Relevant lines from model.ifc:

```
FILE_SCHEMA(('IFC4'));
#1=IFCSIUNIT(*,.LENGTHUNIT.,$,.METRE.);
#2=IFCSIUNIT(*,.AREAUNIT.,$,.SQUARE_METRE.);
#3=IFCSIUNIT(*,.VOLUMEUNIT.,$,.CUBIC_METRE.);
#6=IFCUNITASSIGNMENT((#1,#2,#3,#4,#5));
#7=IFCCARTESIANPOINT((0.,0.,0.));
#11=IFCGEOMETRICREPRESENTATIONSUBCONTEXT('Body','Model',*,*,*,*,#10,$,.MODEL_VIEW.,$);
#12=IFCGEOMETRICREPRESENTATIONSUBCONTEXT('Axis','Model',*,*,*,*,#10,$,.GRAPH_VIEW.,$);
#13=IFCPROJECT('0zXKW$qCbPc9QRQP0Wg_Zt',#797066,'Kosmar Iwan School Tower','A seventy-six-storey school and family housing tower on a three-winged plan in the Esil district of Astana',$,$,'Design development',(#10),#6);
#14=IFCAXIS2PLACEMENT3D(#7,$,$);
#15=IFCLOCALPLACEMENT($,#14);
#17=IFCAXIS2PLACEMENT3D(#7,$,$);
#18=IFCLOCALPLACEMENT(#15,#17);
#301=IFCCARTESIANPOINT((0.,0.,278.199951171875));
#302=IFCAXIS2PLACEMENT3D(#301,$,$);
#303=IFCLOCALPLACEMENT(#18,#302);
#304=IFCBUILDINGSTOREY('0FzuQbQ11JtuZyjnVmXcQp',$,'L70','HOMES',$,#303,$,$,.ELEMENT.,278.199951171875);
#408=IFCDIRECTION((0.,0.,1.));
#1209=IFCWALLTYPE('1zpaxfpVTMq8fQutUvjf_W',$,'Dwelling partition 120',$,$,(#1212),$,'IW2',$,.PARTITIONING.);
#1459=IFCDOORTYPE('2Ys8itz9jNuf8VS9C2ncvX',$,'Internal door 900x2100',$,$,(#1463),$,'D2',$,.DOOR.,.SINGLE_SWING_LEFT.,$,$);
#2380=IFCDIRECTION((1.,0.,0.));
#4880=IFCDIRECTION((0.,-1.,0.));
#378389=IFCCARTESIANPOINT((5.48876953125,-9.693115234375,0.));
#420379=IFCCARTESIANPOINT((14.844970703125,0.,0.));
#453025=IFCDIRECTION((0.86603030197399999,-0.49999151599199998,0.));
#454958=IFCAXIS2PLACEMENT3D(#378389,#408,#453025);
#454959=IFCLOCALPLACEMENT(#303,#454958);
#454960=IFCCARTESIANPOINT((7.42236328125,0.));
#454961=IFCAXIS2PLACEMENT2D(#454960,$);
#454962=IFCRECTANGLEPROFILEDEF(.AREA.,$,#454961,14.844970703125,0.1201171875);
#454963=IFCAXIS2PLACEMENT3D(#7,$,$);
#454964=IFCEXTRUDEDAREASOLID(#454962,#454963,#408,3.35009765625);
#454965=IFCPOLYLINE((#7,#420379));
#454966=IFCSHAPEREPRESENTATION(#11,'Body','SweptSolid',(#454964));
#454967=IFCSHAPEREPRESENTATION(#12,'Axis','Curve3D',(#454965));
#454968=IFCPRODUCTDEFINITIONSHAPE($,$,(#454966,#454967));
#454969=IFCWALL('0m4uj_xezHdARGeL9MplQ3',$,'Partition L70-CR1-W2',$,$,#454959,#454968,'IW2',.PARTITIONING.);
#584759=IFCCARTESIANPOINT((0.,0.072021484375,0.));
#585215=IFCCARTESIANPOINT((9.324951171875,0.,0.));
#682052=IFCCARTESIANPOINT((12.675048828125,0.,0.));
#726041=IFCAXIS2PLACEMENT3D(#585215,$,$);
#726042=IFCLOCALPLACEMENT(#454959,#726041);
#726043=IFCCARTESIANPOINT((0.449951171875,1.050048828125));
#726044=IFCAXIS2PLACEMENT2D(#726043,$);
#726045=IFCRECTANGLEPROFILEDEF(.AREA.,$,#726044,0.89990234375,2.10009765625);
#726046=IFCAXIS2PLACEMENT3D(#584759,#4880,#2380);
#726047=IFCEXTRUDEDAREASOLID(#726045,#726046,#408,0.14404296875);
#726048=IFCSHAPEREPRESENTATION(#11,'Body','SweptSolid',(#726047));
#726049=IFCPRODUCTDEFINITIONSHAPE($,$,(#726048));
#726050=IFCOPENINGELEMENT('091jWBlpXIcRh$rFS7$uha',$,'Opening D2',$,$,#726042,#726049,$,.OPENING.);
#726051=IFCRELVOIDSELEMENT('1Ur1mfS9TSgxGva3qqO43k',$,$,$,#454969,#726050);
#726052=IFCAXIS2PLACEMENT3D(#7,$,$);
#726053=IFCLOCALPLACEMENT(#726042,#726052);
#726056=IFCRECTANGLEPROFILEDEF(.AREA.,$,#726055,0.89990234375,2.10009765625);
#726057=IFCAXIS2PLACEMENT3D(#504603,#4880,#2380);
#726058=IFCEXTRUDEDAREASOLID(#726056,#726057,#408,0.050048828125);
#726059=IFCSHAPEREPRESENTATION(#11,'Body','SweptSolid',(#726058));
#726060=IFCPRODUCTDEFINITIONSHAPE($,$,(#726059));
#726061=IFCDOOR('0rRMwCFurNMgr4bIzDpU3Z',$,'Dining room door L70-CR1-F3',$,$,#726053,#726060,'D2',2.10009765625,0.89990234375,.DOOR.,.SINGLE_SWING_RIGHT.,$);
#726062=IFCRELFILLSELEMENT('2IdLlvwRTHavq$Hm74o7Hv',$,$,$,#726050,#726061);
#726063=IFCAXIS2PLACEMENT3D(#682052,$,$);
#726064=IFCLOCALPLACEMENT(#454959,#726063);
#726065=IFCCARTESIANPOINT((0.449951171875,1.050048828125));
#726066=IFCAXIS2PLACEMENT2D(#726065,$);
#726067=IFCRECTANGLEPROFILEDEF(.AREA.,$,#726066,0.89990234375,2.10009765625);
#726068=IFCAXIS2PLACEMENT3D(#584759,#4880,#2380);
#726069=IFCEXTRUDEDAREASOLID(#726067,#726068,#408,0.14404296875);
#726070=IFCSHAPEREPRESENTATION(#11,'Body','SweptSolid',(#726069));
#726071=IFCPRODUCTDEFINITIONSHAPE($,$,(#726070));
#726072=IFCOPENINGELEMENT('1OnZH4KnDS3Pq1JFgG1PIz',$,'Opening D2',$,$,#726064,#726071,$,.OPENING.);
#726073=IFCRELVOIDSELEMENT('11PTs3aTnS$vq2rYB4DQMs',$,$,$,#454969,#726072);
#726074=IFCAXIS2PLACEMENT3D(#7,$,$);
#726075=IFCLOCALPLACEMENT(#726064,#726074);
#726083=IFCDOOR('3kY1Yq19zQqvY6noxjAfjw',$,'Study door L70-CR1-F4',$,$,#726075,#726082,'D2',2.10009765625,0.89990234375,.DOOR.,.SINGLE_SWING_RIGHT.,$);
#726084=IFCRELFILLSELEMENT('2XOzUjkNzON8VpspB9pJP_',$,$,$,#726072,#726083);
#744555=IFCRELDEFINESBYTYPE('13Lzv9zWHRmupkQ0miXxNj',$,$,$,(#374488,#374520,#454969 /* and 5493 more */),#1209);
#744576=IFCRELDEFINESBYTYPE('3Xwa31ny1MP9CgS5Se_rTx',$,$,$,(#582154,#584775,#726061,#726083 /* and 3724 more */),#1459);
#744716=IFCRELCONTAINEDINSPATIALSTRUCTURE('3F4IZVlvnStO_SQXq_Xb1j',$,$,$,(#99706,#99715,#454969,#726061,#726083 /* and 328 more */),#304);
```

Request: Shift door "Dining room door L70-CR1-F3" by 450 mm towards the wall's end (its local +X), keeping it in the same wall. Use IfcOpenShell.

```python
import ifcopenshell
import ifcopenshell.api.geometry
import ifcopenshell.util.placement
import ifcopenshell.util.unit

model = ifcopenshell.open("model.ifc")
unit_scale = ifcopenshell.util.unit.calculate_unit_scale(model)

door = model.by_guid("0rRMwCFurNMgr4bIzDpU3Z")
opening = door.FillsVoids[0].RelatingOpeningElement
wall = opening.VoidsElements[0].RelatingBuildingElement

wall_matrix = ifcopenshell.util.placement.get_local_placement(wall.ObjectPlacement)
shift = wall_matrix[:3, 0] * 0.45 / unit_scale
before = ifcopenshell.util.placement.get_local_placement(door.ObjectPlacement)[:3, 3].copy()

# The door is placed relative to its opening, so it follows when the opening moves.
matrix = ifcopenshell.util.placement.get_local_placement(opening.ObjectPlacement)
matrix[:3, 3] += shift
ifcopenshell.api.geometry.edit_object_placement(
    model, product=opening, matrix=matrix, is_si=False, should_transform_children=True
)

after = ifcopenshell.util.placement.get_local_placement(door.ObjectPlacement)[:3, 3]
print("door moved by", (after - before).round(3) + 0.0)

model.write("model_rev.ifc")
```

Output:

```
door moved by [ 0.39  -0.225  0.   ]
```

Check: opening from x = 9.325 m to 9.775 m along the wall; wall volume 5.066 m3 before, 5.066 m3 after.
